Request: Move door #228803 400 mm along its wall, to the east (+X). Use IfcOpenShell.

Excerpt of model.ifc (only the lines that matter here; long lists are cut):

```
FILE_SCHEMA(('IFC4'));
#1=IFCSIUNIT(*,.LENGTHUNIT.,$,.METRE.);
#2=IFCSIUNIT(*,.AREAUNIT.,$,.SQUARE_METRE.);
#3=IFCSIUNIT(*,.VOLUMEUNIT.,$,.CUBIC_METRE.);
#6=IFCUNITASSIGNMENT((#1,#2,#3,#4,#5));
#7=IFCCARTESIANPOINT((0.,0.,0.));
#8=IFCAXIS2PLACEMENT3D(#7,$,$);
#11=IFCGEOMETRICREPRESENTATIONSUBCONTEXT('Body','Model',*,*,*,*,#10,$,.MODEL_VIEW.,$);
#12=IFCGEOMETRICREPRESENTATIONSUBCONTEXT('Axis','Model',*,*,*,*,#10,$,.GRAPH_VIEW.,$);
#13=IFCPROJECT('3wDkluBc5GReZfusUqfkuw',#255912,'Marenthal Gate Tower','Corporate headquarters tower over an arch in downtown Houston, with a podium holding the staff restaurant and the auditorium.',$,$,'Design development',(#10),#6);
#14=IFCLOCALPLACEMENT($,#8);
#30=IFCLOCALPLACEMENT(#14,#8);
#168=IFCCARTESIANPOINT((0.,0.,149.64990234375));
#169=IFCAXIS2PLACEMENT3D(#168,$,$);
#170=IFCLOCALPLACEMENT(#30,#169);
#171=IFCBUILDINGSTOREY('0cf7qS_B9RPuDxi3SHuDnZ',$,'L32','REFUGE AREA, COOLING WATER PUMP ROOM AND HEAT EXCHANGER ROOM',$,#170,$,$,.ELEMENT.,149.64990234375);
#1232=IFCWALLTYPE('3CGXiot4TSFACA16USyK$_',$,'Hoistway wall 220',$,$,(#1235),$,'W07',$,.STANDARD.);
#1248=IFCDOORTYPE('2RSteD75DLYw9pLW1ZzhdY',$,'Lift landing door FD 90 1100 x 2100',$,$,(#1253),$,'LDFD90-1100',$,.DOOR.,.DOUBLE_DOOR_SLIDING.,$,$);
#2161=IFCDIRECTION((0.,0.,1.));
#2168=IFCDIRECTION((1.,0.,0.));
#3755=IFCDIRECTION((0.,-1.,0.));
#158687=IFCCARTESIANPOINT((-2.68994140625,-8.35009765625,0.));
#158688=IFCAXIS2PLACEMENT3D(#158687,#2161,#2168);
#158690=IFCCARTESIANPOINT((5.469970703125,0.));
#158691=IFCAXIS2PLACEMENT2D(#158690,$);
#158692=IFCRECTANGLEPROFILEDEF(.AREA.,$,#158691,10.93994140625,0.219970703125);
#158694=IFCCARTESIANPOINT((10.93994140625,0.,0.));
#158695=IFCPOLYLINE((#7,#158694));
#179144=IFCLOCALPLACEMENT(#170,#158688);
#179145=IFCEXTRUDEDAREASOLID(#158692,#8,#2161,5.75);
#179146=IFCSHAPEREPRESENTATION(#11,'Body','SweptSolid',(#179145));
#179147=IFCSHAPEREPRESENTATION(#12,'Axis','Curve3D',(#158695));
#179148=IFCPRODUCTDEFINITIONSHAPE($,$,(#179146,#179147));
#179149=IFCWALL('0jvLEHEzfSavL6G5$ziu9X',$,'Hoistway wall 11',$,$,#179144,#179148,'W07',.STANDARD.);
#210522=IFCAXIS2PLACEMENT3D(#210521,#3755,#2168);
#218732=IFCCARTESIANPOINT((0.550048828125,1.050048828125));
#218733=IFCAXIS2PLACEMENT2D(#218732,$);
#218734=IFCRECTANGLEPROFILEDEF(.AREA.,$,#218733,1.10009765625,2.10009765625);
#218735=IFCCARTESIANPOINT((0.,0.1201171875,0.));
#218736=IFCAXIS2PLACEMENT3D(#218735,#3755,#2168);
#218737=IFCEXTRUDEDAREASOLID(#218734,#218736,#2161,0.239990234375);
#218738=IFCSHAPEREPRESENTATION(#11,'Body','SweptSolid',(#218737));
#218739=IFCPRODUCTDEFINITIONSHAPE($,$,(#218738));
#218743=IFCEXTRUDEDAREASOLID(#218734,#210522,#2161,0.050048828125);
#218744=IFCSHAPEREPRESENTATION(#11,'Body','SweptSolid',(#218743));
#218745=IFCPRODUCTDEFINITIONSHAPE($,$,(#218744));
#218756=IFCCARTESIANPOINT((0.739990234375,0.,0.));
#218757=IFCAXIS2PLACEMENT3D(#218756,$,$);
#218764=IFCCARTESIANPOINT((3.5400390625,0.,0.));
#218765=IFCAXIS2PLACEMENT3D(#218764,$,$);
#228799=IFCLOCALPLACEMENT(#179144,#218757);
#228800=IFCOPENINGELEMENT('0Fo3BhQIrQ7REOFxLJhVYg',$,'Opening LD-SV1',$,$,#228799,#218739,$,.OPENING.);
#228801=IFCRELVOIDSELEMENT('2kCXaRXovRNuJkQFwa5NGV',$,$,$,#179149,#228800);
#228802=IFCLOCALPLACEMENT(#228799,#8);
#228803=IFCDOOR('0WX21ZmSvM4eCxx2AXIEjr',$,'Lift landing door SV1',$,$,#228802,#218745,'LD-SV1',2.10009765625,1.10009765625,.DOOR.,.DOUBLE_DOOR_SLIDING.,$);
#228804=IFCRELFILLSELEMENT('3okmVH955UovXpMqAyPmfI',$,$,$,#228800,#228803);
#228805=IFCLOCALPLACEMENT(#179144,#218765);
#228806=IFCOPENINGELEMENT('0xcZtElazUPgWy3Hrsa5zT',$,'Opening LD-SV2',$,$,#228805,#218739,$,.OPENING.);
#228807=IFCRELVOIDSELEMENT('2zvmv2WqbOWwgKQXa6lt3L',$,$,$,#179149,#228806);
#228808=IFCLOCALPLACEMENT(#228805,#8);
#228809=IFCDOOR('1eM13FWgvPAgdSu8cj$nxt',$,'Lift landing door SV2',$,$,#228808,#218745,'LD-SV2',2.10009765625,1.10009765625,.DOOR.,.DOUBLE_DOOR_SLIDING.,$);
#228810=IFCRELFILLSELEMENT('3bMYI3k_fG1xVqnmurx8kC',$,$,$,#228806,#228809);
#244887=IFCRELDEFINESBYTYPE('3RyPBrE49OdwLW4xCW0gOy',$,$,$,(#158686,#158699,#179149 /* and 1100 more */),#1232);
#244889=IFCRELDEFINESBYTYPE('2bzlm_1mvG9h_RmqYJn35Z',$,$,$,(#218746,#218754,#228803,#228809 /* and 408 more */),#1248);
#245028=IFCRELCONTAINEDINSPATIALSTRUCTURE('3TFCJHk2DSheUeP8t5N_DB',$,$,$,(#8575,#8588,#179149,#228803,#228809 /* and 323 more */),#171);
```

```python
import ifcopenshell
import ifcopenshell.api.geometry
import ifcopenshell.util.placement

model = ifcopenshell.open("model.ifc")

door = model.by_id(228803)
opening = door.FillsVoids[0].RelatingOpeningElement
wall = opening.VoidsElements[0].RelatingBuildingElement

wall_matrix = ifcopenshell.util.placement.get_local_placement(wall.ObjectPlacement)
shift = wall_matrix[:3, 0] * 0.4
before = ifcopenshell.util.placement.get_local_placement(door.ObjectPlacement)[:3, 3].copy()

# The door is placed relative to its opening, so it follows when the opening moves.
matrix = ifcopenshell.util.placement.get_local_placement(opening.ObjectPlacement)
matrix[:3, 3] += shift
ifcopenshell.api.geometry.edit_object_placement(
    model, product=opening, matrix=matrix, is_si=False, should_transform_children=True
)

after = ifcopenshell.util.placement.get_local_placement(door.ObjectPlacement)[:3, 3]
print("door moved by", (after - before).round(3) + 0.0)

model.write("model_v2.ifc")
```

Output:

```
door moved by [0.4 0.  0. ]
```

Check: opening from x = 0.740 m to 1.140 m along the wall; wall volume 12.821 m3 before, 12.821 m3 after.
